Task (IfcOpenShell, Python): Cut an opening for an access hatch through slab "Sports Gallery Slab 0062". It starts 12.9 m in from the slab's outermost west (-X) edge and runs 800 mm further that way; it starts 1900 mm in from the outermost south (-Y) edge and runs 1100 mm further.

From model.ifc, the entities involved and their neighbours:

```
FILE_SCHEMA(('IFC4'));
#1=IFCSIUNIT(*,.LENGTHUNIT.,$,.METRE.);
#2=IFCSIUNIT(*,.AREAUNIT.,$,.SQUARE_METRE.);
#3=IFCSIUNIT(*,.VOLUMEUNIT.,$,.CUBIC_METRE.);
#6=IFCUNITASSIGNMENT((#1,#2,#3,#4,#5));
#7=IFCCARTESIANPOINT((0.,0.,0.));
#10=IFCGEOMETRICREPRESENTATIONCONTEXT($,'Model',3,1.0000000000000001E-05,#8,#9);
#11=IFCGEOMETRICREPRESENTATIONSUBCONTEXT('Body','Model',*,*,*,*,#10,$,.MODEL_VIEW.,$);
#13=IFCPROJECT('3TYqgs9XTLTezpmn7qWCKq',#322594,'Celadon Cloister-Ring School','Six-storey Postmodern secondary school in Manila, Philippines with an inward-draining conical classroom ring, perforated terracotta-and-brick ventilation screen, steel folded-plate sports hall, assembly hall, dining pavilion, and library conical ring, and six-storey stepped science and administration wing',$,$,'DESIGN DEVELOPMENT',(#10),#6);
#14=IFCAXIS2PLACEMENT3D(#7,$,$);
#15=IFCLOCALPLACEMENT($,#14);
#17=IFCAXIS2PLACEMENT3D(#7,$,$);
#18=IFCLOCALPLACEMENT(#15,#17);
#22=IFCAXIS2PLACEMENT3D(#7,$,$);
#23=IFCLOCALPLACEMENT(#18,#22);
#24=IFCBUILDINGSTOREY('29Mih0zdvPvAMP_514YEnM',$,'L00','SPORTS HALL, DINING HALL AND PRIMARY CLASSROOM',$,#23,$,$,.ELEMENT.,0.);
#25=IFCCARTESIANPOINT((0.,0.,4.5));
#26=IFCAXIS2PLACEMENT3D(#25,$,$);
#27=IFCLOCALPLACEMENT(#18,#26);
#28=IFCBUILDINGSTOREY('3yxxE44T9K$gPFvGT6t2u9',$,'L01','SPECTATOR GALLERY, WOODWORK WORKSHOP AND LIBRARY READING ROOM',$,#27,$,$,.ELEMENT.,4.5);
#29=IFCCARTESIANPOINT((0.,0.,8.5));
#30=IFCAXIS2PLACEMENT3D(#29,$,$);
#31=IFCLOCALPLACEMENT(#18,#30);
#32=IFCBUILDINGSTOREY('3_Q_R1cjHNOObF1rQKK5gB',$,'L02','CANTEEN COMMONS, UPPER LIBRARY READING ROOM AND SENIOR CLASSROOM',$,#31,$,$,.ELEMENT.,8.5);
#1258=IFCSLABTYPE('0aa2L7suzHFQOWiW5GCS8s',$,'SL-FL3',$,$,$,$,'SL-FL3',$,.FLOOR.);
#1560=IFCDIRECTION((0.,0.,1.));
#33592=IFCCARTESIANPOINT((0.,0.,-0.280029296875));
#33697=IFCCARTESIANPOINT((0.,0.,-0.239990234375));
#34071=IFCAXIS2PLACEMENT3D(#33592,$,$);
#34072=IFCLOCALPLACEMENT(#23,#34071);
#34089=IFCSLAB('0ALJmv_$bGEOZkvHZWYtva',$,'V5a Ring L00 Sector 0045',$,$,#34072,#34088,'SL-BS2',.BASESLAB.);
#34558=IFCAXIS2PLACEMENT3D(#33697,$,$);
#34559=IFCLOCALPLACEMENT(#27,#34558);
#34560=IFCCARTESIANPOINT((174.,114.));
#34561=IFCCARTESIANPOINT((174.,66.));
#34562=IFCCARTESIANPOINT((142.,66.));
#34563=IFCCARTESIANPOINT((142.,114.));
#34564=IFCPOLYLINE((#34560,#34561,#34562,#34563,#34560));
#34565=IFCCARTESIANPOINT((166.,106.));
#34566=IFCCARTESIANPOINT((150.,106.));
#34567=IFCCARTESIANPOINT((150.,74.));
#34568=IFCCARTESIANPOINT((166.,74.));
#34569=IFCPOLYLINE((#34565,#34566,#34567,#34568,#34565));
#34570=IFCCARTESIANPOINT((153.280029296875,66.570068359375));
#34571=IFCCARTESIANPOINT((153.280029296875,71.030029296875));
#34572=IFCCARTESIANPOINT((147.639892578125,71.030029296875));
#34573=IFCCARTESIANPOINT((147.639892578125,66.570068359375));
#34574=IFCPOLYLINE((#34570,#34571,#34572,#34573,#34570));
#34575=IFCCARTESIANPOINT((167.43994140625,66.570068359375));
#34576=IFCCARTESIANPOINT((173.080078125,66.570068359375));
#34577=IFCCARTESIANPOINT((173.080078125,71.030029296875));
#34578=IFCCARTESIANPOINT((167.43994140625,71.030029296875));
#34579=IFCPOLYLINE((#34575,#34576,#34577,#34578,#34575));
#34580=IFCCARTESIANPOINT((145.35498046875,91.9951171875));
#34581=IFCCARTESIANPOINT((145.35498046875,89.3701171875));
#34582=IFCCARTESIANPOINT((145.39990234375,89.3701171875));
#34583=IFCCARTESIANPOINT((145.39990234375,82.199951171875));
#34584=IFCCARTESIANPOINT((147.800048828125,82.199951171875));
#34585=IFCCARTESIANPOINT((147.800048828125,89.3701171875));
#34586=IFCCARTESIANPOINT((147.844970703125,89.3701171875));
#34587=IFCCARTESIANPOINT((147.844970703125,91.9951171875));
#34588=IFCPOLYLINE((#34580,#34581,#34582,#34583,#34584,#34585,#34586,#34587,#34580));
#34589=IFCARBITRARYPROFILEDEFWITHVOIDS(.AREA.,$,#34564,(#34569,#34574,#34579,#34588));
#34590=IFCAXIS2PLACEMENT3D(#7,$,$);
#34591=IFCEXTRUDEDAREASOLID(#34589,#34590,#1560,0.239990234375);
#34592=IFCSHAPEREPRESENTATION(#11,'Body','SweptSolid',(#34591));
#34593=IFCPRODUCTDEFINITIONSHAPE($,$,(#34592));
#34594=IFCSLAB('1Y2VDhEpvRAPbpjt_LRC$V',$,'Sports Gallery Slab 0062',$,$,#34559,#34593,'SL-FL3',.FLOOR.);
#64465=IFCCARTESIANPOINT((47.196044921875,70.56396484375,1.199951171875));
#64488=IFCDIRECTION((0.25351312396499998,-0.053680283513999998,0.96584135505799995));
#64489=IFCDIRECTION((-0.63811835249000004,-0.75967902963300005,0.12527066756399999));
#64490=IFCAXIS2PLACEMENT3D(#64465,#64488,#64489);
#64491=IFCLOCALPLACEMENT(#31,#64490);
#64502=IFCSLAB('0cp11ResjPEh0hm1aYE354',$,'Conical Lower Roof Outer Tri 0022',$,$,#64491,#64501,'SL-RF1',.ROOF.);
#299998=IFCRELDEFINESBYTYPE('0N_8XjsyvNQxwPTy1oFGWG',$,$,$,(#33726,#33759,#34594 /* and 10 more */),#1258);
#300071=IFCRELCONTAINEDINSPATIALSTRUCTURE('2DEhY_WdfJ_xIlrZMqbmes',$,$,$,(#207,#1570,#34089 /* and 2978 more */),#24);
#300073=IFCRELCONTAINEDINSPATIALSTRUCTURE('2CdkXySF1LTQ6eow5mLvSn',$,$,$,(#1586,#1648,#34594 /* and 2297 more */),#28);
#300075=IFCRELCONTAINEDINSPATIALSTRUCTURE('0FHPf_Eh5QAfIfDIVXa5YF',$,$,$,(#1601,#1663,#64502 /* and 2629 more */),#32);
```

```python
import numpy as np
import ifcopenshell
import ifcopenshell.api.feature
import ifcopenshell.api.geometry
import ifcopenshell.api.root
import ifcopenshell.geom
import ifcopenshell.util.placement
import ifcopenshell.util.representation
import ifcopenshell.util.shape
import ifcopenshell.util.unit

model = ifcopenshell.open("model.ifc")
unit_scale = ifcopenshell.util.unit.calculate_unit_scale(model)
settings = ifcopenshell.geom.settings()


def volume(element):
    """Net volume in cubic metres, openings subtracted."""
    shape = ifcopenshell.geom.create_shape(settings, element)
    return ifcopenshell.util.shape.get_volume(shape.geometry)


slab = model.by_guid("1Y2VDhEpvRAPbpjt_LRC$V")
before = volume(slab)

# Extent in the slab's own axes, in metres. The edges named are its -X and -Y sides.
slab_shape = ifcopenshell.geom.create_shape(settings, slab)
vertices = ifcopenshell.util.shape.get_vertices(slab_shape.geometry)
x_min, y_min, bottom = vertices.min(axis=0)
top = vertices[:, 2].max()

opening = ifcopenshell.api.root.create_entity(model, ifc_class="IfcOpeningElement", name="Access hatch opening", predefined_type="OPENING")
context = ifcopenshell.util.representation.get_context(model, "Model", "Body", "MODEL_VIEW")
width, depth = 0.8, 1.1
outline = [(0.0, 0.0), (width, 0.0), (width, depth), (0.0, depth), (0.0, 0.0)]
# Overshoot both faces by 50 mm so the cut is clean.
shape = ifcopenshell.api.geometry.add_slab_representation(
    model, context=context, depth=top - bottom + 0.1, polyline=outline
)
ifcopenshell.api.geometry.assign_representation(model, product=opening, representation=shape)

matrix = ifcopenshell.util.placement.get_local_placement(slab.ObjectPlacement)
matrix[:, 3] = matrix @ np.append(np.array([x_min + 12.9, y_min + 1.9, bottom - 0.05]) / unit_scale, 1.0)
ifcopenshell.api.geometry.edit_object_placement(model, product=opening, matrix=matrix, is_si=False)
ifcopenshell.api.feature.add_feature(model, feature=opening, element=slab)

after = volume(slab)

print(f"slab volume {before:.3f} -> {after:.3f} m3")

model.write("model_rev.ifc")
```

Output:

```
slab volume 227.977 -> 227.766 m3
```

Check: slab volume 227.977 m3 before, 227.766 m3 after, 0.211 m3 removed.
